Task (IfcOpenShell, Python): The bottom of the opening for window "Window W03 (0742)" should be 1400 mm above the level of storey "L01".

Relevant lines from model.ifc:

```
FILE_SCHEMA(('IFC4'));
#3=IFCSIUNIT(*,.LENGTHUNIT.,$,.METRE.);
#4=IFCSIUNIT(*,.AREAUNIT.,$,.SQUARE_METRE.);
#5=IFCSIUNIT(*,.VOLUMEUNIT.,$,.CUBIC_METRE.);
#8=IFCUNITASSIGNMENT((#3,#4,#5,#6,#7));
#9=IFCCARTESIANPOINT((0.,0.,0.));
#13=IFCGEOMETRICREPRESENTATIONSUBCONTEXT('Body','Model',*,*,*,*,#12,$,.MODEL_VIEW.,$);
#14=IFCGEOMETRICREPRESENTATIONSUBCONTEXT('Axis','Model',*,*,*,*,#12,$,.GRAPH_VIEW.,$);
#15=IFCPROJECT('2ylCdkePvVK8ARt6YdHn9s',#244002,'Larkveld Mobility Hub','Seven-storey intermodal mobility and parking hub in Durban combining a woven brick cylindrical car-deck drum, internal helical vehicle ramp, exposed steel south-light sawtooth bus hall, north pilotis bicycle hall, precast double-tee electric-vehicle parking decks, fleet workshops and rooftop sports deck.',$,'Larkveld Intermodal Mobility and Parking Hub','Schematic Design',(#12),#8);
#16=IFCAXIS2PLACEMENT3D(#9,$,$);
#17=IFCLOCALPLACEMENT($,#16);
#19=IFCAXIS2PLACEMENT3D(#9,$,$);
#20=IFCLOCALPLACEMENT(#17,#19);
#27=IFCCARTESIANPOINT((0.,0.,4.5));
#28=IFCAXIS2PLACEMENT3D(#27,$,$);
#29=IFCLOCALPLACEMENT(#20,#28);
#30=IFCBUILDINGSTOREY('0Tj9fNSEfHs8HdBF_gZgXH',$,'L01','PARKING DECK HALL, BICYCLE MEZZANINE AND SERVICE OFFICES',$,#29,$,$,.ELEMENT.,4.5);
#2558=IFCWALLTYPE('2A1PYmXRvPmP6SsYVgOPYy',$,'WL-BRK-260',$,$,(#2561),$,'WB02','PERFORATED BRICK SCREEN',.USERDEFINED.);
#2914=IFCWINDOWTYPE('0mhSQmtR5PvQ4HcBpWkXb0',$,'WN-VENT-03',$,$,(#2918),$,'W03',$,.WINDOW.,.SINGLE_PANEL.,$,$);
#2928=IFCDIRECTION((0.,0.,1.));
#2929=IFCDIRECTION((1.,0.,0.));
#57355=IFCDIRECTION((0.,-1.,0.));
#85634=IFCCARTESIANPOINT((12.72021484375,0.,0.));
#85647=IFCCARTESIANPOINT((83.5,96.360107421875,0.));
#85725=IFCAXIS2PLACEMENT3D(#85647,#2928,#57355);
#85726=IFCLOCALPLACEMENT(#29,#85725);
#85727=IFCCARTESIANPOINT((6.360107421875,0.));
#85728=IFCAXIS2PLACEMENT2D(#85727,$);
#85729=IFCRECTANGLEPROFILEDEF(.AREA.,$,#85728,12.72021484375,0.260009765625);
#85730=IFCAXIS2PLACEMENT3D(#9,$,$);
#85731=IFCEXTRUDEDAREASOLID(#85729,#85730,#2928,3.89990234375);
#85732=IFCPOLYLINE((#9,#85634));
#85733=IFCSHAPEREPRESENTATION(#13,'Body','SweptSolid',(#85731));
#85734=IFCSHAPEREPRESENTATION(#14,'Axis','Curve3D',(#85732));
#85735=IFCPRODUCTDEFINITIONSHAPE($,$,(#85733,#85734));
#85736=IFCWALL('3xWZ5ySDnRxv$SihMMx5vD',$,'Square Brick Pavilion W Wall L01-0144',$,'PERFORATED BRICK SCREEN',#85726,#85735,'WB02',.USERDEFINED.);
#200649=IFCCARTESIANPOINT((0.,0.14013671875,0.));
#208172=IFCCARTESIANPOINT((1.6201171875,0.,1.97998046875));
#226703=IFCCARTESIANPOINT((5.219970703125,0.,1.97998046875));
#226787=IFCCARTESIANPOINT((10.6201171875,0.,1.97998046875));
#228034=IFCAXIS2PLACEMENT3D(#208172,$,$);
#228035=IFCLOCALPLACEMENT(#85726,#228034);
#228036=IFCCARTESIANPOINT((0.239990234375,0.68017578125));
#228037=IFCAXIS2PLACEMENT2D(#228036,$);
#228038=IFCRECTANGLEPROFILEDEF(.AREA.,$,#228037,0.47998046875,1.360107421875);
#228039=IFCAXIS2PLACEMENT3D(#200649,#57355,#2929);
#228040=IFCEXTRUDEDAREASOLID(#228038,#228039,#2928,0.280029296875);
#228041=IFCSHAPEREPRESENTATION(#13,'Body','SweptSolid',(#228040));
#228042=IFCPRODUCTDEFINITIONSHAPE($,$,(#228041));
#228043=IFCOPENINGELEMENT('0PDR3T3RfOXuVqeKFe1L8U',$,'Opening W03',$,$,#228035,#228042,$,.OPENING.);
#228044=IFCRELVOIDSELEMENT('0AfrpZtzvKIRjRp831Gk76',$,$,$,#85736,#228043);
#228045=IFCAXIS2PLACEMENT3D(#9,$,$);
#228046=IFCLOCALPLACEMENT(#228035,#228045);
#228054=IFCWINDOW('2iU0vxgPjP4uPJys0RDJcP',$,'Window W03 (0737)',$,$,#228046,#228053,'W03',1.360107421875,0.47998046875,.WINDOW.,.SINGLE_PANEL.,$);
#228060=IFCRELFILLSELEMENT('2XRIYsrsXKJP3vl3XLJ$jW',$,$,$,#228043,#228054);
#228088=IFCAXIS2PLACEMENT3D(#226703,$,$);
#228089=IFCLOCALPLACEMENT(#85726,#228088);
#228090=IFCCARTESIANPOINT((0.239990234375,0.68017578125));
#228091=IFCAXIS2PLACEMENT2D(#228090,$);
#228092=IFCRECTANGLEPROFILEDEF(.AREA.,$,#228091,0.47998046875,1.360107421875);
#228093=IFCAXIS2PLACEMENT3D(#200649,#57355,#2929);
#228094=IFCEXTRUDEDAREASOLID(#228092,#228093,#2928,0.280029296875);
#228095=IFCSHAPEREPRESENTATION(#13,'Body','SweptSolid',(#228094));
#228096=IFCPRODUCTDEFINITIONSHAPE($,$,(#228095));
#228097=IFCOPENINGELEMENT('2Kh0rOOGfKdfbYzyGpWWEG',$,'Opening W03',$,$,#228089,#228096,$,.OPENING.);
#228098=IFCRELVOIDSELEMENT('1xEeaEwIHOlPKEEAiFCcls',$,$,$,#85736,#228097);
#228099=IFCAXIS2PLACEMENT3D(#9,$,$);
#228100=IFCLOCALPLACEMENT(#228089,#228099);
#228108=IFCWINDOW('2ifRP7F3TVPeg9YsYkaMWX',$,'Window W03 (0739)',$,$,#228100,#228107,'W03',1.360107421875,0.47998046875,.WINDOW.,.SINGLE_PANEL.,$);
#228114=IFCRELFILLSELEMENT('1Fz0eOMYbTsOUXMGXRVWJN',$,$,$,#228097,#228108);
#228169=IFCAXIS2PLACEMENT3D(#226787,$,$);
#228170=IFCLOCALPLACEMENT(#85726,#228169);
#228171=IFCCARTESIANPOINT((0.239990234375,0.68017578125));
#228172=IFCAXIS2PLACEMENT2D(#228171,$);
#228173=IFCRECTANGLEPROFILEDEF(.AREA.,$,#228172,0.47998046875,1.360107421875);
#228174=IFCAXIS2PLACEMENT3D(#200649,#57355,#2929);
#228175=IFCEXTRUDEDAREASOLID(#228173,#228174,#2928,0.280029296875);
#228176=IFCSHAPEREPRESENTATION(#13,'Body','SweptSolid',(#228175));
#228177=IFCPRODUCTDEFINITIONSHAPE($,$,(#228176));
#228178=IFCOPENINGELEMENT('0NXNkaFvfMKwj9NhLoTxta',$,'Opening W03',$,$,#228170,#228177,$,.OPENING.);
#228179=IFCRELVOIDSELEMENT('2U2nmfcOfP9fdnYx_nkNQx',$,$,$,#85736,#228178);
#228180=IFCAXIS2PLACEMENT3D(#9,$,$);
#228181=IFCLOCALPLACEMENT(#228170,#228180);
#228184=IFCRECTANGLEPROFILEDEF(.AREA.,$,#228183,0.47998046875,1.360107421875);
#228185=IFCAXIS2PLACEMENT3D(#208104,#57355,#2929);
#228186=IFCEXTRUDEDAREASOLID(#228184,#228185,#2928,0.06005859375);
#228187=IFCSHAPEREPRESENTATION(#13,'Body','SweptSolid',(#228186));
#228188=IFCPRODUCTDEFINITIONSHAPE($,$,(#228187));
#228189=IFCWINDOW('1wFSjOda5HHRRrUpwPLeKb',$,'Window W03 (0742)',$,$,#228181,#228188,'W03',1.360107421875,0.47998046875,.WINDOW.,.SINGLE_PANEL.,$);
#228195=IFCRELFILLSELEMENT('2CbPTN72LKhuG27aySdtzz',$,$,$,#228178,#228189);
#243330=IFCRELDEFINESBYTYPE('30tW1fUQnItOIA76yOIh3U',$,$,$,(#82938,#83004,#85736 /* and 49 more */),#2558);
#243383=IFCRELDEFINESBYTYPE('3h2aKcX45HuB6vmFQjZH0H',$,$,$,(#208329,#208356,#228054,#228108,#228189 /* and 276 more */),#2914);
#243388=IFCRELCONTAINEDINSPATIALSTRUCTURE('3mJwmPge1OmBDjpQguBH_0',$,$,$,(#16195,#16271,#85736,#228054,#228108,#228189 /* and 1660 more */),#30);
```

```python
import numpy as np
import ifcopenshell
import ifcopenshell.api.geometry
import ifcopenshell.geom
import ifcopenshell.util.element
import ifcopenshell.util.placement
import ifcopenshell.util.shape
import ifcopenshell.util.unit

model = ifcopenshell.open("model.ifc")
unit_scale = ifcopenshell.util.unit.calculate_unit_scale(model)

window = model.by_guid("1wFSjOda5HHRRrUpwPLeKb")
opening = window.FillsVoids[0].RelatingOpeningElement
storey = ifcopenshell.util.element.get_container(window, ifc_class="IfcBuildingStorey")
level = ifcopenshell.util.placement.get_local_placement(storey.ObjectPlacement)[2, 3]

# The opening's origin need not be at the sill, so measure its lowest point.
shape = ifcopenshell.geom.create_shape(ifcopenshell.geom.settings(), opening)
bottom = ifcopenshell.util.shape.get_shape_bottom_elevation(shape, shape.geometry) / unit_scale
dz = level + 1.4 / unit_scale - bottom

shift = np.array([0.0, 0.0, dz])
# The window is placed relative to its opening, so it follows when the opening moves.
matrix = ifcopenshell.util.placement.get_local_placement(opening.ObjectPlacement)
matrix[:3, 3] += shift
ifcopenshell.api.geometry.edit_object_placement(
    model, product=opening, matrix=matrix, is_si=False, should_transform_children=True
)

print(f"moved by {dz * unit_scale:+.3f} m")

model.write("model_updated.ifc")
```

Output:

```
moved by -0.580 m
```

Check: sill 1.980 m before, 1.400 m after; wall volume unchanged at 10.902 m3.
